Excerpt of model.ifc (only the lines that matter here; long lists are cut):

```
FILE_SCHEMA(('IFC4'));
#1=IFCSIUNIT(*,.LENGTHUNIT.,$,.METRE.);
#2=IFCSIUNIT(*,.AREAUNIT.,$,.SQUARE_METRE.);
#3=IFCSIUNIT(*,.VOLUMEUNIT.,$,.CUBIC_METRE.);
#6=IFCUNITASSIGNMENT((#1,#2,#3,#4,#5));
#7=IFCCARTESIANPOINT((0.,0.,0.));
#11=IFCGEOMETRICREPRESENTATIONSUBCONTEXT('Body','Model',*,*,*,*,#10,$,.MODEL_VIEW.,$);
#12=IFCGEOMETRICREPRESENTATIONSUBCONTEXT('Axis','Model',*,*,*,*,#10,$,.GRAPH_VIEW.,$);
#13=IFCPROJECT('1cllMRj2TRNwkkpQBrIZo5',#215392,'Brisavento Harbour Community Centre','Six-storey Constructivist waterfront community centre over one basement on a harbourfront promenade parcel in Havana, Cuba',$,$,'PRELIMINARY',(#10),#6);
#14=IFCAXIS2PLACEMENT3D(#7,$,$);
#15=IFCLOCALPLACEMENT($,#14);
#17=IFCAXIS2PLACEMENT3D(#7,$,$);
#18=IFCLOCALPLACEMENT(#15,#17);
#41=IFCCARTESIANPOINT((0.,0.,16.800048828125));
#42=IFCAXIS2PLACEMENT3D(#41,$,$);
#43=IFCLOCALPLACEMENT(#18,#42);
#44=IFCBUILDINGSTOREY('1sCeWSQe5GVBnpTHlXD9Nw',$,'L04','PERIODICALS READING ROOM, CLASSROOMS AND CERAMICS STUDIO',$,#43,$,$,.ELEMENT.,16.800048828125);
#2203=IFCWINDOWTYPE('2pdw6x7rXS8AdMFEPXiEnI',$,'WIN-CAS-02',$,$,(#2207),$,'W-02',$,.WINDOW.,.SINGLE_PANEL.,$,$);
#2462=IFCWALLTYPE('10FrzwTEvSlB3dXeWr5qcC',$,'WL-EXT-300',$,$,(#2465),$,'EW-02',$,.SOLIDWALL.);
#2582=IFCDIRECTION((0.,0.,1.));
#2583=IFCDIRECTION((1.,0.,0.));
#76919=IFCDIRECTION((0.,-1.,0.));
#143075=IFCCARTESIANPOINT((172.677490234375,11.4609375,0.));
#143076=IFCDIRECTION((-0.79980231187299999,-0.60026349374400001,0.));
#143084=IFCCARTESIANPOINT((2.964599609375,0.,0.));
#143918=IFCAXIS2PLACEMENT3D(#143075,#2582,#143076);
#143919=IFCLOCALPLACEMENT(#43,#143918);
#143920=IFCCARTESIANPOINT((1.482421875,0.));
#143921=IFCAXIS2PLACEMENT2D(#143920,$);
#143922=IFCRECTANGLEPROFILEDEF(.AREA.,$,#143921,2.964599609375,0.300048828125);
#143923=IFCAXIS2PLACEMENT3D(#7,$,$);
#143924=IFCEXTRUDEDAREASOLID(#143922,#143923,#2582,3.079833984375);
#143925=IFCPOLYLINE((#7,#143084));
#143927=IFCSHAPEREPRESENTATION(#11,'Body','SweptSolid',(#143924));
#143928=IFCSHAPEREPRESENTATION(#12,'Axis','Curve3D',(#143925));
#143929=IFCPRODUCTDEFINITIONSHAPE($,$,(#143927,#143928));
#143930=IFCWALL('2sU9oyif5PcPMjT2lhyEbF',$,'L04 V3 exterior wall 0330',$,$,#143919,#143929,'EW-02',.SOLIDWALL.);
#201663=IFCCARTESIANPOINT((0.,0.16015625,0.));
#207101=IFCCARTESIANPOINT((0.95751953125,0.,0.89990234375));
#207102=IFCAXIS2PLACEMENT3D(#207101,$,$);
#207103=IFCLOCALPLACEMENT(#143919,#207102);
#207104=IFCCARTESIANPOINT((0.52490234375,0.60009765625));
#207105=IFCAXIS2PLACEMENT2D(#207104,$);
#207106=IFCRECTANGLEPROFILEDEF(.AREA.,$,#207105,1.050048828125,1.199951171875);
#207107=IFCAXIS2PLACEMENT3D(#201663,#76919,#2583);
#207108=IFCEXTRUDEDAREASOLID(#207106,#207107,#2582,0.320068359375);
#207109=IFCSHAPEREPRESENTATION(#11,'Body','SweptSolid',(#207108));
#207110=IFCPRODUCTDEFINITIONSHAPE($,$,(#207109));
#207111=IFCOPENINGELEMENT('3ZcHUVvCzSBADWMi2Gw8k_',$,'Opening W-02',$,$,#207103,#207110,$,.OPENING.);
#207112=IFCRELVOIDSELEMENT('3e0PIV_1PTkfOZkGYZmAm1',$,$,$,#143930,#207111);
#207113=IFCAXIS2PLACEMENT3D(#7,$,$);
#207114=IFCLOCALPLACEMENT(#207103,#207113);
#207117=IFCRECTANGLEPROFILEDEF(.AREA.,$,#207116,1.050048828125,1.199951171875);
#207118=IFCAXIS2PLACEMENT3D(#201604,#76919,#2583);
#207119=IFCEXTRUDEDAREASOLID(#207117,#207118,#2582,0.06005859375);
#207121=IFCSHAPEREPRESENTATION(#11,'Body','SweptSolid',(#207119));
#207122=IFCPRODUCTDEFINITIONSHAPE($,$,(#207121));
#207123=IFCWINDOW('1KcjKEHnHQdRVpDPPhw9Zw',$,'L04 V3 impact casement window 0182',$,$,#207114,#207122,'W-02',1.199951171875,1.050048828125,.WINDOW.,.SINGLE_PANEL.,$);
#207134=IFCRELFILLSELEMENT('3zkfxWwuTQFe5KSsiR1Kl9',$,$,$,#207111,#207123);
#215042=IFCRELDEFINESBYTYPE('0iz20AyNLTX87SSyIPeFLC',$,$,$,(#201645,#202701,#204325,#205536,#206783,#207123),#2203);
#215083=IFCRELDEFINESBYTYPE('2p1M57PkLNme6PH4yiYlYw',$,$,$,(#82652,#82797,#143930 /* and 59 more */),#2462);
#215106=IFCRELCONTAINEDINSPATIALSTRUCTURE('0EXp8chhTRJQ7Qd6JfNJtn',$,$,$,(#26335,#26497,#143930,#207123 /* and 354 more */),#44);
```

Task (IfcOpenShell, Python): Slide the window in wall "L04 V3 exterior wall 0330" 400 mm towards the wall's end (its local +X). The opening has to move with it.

```python
import ifcopenshell
import ifcopenshell.api.geometry
import ifcopenshell.util.placement
import ifcopenshell.util.unit

model = ifcopenshell.open("model.ifc")
unit_scale = ifcopenshell.util.unit.calculate_unit_scale(model)

window = model.by_id(207123)
opening = window.FillsVoids[0].RelatingOpeningElement
wall = opening.VoidsElements[0].RelatingBuildingElement

wall_matrix = ifcopenshell.util.placement.get_local_placement(wall.ObjectPlacement)
shift = wall_matrix[:3, 0] * 0.4 / unit_scale
before = ifcopenshell.util.placement.get_local_placement(window.ObjectPlacement)[:3, 3].copy()

# The window is placed relative to its opening, so it follows when the opening moves.
matrix = ifcopenshell.util.placement.get_local_placement(opening.ObjectPlacement)
matrix[:3, 3] += shift
ifcopenshell.api.geometry.edit_object_placement(
    model, product=opening, matrix=matrix, is_si=False, should_transform_children=True
)

after = ifcopenshell.util.placement.get_local_placement(window.ObjectPlacement)[:3, 3]
print("window moved by", (after - before).round(3) + 0.0)

model.write("model-out.ifc")
```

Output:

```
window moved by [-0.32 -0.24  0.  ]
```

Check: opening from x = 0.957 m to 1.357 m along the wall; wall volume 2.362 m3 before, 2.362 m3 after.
